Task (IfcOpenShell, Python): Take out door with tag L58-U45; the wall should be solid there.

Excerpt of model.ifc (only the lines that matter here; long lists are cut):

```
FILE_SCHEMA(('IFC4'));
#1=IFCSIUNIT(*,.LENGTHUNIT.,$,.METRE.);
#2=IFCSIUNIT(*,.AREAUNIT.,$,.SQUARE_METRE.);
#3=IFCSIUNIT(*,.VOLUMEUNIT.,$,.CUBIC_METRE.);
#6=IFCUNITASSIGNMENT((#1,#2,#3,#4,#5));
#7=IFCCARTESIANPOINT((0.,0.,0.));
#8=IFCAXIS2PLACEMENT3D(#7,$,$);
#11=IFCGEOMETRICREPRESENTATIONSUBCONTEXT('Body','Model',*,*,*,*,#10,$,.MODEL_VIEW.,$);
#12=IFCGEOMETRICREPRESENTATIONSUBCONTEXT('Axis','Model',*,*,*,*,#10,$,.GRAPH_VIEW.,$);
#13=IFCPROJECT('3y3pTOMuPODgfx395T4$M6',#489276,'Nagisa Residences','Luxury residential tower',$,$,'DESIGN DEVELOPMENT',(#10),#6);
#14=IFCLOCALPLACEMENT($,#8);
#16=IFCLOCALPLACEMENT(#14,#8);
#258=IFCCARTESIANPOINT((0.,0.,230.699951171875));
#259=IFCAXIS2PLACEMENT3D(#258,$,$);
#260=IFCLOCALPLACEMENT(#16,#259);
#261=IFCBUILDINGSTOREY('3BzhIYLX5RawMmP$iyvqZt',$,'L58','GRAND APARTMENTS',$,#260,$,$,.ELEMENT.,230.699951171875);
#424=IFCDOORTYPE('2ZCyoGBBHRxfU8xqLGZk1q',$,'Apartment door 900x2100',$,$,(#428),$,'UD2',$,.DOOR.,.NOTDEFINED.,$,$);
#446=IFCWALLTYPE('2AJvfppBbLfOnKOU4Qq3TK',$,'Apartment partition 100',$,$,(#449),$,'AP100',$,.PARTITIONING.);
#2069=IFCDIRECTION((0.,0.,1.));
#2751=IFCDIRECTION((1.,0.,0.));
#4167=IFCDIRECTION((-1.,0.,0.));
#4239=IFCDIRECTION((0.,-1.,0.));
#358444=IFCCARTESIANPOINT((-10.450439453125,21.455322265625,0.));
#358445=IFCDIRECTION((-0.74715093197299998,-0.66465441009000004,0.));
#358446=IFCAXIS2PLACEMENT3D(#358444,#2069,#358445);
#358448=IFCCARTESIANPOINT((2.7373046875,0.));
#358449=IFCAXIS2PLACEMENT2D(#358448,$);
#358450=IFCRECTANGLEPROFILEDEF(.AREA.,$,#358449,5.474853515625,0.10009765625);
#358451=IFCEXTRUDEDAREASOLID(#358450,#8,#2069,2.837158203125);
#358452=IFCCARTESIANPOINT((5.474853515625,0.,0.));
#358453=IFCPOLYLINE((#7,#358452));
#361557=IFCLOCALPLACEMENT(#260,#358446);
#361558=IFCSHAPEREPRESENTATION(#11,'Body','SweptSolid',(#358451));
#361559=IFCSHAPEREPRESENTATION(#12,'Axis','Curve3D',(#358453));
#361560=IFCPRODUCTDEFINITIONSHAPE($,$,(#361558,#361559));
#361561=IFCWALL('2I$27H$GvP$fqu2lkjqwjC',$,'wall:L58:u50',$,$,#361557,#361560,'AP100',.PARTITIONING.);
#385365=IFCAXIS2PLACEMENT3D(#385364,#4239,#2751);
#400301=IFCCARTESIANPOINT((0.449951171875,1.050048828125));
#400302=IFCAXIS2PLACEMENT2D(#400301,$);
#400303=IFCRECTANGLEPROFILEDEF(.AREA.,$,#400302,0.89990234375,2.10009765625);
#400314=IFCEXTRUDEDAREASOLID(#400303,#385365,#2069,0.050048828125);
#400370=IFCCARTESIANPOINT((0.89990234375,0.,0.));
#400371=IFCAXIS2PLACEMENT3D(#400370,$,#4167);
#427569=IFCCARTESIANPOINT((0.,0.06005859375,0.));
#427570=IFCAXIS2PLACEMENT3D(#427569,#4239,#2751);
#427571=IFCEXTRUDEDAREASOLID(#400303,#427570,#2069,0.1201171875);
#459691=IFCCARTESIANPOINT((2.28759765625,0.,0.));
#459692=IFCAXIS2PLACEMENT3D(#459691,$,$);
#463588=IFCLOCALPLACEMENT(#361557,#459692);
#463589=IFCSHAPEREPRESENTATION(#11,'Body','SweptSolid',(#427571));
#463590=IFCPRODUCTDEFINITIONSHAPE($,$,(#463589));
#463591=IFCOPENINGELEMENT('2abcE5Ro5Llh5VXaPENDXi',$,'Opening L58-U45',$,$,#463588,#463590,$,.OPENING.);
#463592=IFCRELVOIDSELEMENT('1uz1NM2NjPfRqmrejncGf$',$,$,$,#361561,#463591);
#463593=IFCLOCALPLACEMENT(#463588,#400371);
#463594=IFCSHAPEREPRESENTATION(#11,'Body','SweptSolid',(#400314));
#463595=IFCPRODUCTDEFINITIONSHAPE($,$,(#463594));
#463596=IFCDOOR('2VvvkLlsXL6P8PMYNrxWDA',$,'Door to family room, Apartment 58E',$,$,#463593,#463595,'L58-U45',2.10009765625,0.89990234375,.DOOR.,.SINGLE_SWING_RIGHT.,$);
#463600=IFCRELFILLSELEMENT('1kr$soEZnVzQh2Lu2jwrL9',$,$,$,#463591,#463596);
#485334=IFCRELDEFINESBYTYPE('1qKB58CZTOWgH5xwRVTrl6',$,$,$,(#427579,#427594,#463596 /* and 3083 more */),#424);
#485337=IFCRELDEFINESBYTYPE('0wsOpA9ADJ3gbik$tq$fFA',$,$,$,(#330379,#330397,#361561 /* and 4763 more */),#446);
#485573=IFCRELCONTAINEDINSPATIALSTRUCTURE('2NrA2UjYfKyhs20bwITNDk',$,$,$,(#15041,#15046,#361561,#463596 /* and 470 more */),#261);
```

```python
import ifcopenshell
import ifcopenshell.api.feature
import ifcopenshell.api.root
import ifcopenshell.geom
import ifcopenshell.util.shape

model = ifcopenshell.open("model.ifc")
settings = ifcopenshell.geom.settings()


def volume(element):
    """Net volume in cubic metres, openings subtracted."""
    shape = ifcopenshell.geom.create_shape(settings, element)
    return ifcopenshell.util.shape.get_volume(shape.geometry)


door = model.by_guid("2VvvkLlsXL6P8PMYNrxWDA")
opening = door.FillsVoids[0].RelatingOpeningElement
wall = opening.VoidsElements[0].RelatingBuildingElement
before = volume(wall)

ifcopenshell.api.root.remove_product(model, product=door)
ifcopenshell.api.feature.remove_feature(model, feature=opening)

after = volume(wall)

print(f"wall volume {before:.3f} -> {after:.3f} m3")

model.write("model_v2.ifc")
```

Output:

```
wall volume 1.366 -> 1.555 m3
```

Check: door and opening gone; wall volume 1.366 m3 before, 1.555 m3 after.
